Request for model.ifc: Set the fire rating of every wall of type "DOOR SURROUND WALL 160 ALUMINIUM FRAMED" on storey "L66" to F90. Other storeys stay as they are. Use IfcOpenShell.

First a look at what the model holds.

```python
import ifcopenshell
import ifcopenshell.util.element

model = ifcopenshell.open("model.ifc")
print(model.schema)
storey = next(s for s in model.by_type("IfcBuildingStorey") if s.Name == "L66")
walls = [e for e in ifcopenshell.util.element.get_decomposition(storey) if e.is_a("IfcWall")]
seen = {}
for e in walls:
    element_type = ifcopenshell.util.element.get_type(e)
    key = (element_type.Name if element_type != e and element_type else None, ifcopenshell.util.element.get_pset(e, "Pset_WallCommon", "FireRating"))
    seen[key] = seen.get(key, 0) + 1
for (name, value), count in sorted(seen.items(), key=str):
    print(count, "x", name, "|", value)
```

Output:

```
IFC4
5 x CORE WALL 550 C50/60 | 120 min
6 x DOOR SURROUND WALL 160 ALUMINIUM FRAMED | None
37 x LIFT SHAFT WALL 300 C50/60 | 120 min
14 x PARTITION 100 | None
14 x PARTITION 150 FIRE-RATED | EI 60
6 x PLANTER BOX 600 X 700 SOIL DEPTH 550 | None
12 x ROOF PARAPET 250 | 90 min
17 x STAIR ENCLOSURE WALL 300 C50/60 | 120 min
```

```python
import ifcopenshell
import ifcopenshell.api.pset
import ifcopenshell.util.element

model = ifcopenshell.open("model.ifc")

storey = next(s for s in model.by_type("IfcBuildingStorey") if s.Name == "L66")
walls = [e for e in ifcopenshell.util.element.get_decomposition(storey) if e.is_a("IfcWall")]

count = 0
for e in walls:
    element_type = ifcopenshell.util.element.get_type(e)
    if element_type in (None, e) or element_type.Name != "DOOR SURROUND WALL 160 ALUMINIUM FRAMED":
        continue
    found = ifcopenshell.util.element.get_pset(e, "Pset_WallCommon", should_inherit=False)
    if found:
        pset = model.by_id(found["id"])
        if len(ifcopenshell.util.element.get_elements_by_pset(pset)) > 1:
            pset = ifcopenshell.api.pset.unshare_pset(model, products=[e], pset=pset)[0]
    else:
        pset = ifcopenshell.api.pset.add_pset(model, product=e, name="Pset_WallCommon")
    ifcopenshell.api.pset.edit_pset(model, pset=pset, properties={"FireRating": "F90"})
    count += 1

print(count, "walls updated")

model.write("model-out.ifc")
```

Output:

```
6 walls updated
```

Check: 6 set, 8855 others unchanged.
